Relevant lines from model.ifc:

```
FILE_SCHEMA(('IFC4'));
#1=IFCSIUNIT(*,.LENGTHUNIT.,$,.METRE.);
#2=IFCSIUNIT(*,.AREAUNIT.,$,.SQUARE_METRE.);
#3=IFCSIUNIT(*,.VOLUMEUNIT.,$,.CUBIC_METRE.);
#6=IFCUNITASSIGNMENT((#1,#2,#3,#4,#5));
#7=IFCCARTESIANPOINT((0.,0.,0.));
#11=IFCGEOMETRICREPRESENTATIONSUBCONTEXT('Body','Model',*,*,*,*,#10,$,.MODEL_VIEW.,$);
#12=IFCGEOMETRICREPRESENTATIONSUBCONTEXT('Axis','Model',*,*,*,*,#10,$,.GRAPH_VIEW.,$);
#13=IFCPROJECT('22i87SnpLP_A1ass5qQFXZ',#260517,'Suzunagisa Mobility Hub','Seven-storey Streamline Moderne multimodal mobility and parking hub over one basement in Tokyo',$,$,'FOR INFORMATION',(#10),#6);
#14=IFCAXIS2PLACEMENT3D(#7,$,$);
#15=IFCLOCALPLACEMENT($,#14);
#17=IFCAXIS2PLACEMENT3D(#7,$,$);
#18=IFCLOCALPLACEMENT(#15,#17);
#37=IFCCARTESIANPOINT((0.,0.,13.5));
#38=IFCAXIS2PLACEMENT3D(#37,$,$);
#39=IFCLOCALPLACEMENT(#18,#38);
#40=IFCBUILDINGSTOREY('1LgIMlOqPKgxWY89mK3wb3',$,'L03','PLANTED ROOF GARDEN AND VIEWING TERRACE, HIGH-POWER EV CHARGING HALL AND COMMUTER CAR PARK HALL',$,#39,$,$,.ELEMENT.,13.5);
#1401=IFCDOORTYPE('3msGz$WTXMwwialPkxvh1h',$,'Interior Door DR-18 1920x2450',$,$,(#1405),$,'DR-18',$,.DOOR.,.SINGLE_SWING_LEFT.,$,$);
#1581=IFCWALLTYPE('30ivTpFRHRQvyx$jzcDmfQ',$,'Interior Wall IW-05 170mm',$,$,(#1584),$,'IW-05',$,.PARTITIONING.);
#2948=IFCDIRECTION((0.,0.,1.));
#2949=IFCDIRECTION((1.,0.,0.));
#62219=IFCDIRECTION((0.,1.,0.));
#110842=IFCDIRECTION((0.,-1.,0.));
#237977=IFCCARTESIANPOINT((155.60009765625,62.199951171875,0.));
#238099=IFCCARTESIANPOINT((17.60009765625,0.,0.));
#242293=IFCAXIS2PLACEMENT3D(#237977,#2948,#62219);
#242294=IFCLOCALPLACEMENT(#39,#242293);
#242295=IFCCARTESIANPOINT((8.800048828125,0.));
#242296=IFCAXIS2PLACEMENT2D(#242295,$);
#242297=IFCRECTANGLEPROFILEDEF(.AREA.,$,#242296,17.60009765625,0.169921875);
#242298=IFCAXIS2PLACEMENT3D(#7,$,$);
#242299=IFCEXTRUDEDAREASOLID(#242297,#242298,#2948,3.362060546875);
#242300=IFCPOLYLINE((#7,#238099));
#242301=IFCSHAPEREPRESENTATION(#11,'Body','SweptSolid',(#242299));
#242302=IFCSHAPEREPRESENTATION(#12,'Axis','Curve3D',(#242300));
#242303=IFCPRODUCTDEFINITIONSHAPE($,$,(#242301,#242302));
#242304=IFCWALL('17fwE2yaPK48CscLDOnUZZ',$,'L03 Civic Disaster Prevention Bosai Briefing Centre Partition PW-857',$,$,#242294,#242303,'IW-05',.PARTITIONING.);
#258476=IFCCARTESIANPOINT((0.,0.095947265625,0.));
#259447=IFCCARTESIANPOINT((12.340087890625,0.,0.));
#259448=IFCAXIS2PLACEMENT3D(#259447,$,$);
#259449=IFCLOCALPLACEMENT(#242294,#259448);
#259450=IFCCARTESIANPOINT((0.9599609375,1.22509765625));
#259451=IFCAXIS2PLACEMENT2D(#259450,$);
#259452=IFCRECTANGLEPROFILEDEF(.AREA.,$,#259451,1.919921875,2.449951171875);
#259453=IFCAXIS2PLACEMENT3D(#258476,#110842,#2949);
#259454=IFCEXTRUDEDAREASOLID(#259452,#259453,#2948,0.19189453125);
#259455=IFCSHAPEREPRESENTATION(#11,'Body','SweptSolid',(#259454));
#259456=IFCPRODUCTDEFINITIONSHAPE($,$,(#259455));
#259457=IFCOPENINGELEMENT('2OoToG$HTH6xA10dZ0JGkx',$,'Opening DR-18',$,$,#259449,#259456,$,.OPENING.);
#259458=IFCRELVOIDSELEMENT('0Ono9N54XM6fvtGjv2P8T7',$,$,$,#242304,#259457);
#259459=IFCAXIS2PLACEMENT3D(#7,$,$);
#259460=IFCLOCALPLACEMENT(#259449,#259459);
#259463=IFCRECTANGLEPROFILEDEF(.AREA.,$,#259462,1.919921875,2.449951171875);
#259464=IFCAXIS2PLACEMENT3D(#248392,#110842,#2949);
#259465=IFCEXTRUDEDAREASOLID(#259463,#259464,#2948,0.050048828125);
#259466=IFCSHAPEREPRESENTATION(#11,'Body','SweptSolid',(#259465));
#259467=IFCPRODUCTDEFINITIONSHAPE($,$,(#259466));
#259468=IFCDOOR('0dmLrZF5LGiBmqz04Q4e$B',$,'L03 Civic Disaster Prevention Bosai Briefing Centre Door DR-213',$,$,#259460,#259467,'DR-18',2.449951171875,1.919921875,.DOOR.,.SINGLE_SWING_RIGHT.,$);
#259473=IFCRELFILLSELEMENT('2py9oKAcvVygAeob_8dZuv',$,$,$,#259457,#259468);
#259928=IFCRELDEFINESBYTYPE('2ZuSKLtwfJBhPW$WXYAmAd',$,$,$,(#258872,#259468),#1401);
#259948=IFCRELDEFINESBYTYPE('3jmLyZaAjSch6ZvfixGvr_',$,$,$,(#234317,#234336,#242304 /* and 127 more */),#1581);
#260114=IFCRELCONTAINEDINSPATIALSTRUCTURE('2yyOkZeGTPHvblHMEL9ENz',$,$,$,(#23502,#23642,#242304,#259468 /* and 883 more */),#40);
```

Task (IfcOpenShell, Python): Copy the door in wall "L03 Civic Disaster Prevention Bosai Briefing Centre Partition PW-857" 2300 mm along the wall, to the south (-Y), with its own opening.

```python
import ifcopenshell
import ifcopenshell.api.feature
import ifcopenshell.api.geometry
import ifcopenshell.api.root
import ifcopenshell.geom
import ifcopenshell.util.element
import ifcopenshell.util.placement
import ifcopenshell.util.shape
import ifcopenshell.util.unit

model = ifcopenshell.open("model.ifc")
unit_scale = ifcopenshell.util.unit.calculate_unit_scale(model)
settings = ifcopenshell.geom.settings()


def volume(element):
    """Net volume in cubic metres, openings subtracted."""
    shape = ifcopenshell.geom.create_shape(settings, element)
    return ifcopenshell.util.shape.get_volume(shape.geometry)


door = model.by_guid("0dmLrZF5LGiBmqz04Q4e$B")
opening = door.FillsVoids[0].RelatingOpeningElement
wall = opening.VoidsElements[0].RelatingBuildingElement
before = volume(wall)
shift = ifcopenshell.util.placement.get_local_placement(wall.ObjectPlacement)[:3, 0] * -2.3 / unit_scale

# copy_class copies the void relationship, type, container and properties, but no geometry.
new_opening = ifcopenshell.api.root.copy_class(model, product=opening)
new_opening.Representation = ifcopenshell.util.element.copy_deep(
    model, opening.Representation, exclude=["IfcGeometricRepresentationContext", "IfcRepresentationMap"]
)
new_door = ifcopenshell.api.root.copy_class(model, product=door)
new_door.Representation = ifcopenshell.util.element.copy_deep(
    model, door.Representation, exclude=["IfcGeometricRepresentationContext", "IfcRepresentationMap"]
)
new_door.Tag = None
ifcopenshell.api.feature.add_filling(model, opening=new_opening, element=new_door)

for old, new in ((opening, new_opening), (door, new_door)):
    matrix = ifcopenshell.util.placement.get_local_placement(old.ObjectPlacement)
    matrix[:3, 3] += shift
    ifcopenshell.api.geometry.edit_object_placement(model, product=new, matrix=matrix, is_si=False)

after = volume(wall)

print(f"wall volume {before:.3f} -> {after:.3f} m3")

model.write("model_updated.ifc")
```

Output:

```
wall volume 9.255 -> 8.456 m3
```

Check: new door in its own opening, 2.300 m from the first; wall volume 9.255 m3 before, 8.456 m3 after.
